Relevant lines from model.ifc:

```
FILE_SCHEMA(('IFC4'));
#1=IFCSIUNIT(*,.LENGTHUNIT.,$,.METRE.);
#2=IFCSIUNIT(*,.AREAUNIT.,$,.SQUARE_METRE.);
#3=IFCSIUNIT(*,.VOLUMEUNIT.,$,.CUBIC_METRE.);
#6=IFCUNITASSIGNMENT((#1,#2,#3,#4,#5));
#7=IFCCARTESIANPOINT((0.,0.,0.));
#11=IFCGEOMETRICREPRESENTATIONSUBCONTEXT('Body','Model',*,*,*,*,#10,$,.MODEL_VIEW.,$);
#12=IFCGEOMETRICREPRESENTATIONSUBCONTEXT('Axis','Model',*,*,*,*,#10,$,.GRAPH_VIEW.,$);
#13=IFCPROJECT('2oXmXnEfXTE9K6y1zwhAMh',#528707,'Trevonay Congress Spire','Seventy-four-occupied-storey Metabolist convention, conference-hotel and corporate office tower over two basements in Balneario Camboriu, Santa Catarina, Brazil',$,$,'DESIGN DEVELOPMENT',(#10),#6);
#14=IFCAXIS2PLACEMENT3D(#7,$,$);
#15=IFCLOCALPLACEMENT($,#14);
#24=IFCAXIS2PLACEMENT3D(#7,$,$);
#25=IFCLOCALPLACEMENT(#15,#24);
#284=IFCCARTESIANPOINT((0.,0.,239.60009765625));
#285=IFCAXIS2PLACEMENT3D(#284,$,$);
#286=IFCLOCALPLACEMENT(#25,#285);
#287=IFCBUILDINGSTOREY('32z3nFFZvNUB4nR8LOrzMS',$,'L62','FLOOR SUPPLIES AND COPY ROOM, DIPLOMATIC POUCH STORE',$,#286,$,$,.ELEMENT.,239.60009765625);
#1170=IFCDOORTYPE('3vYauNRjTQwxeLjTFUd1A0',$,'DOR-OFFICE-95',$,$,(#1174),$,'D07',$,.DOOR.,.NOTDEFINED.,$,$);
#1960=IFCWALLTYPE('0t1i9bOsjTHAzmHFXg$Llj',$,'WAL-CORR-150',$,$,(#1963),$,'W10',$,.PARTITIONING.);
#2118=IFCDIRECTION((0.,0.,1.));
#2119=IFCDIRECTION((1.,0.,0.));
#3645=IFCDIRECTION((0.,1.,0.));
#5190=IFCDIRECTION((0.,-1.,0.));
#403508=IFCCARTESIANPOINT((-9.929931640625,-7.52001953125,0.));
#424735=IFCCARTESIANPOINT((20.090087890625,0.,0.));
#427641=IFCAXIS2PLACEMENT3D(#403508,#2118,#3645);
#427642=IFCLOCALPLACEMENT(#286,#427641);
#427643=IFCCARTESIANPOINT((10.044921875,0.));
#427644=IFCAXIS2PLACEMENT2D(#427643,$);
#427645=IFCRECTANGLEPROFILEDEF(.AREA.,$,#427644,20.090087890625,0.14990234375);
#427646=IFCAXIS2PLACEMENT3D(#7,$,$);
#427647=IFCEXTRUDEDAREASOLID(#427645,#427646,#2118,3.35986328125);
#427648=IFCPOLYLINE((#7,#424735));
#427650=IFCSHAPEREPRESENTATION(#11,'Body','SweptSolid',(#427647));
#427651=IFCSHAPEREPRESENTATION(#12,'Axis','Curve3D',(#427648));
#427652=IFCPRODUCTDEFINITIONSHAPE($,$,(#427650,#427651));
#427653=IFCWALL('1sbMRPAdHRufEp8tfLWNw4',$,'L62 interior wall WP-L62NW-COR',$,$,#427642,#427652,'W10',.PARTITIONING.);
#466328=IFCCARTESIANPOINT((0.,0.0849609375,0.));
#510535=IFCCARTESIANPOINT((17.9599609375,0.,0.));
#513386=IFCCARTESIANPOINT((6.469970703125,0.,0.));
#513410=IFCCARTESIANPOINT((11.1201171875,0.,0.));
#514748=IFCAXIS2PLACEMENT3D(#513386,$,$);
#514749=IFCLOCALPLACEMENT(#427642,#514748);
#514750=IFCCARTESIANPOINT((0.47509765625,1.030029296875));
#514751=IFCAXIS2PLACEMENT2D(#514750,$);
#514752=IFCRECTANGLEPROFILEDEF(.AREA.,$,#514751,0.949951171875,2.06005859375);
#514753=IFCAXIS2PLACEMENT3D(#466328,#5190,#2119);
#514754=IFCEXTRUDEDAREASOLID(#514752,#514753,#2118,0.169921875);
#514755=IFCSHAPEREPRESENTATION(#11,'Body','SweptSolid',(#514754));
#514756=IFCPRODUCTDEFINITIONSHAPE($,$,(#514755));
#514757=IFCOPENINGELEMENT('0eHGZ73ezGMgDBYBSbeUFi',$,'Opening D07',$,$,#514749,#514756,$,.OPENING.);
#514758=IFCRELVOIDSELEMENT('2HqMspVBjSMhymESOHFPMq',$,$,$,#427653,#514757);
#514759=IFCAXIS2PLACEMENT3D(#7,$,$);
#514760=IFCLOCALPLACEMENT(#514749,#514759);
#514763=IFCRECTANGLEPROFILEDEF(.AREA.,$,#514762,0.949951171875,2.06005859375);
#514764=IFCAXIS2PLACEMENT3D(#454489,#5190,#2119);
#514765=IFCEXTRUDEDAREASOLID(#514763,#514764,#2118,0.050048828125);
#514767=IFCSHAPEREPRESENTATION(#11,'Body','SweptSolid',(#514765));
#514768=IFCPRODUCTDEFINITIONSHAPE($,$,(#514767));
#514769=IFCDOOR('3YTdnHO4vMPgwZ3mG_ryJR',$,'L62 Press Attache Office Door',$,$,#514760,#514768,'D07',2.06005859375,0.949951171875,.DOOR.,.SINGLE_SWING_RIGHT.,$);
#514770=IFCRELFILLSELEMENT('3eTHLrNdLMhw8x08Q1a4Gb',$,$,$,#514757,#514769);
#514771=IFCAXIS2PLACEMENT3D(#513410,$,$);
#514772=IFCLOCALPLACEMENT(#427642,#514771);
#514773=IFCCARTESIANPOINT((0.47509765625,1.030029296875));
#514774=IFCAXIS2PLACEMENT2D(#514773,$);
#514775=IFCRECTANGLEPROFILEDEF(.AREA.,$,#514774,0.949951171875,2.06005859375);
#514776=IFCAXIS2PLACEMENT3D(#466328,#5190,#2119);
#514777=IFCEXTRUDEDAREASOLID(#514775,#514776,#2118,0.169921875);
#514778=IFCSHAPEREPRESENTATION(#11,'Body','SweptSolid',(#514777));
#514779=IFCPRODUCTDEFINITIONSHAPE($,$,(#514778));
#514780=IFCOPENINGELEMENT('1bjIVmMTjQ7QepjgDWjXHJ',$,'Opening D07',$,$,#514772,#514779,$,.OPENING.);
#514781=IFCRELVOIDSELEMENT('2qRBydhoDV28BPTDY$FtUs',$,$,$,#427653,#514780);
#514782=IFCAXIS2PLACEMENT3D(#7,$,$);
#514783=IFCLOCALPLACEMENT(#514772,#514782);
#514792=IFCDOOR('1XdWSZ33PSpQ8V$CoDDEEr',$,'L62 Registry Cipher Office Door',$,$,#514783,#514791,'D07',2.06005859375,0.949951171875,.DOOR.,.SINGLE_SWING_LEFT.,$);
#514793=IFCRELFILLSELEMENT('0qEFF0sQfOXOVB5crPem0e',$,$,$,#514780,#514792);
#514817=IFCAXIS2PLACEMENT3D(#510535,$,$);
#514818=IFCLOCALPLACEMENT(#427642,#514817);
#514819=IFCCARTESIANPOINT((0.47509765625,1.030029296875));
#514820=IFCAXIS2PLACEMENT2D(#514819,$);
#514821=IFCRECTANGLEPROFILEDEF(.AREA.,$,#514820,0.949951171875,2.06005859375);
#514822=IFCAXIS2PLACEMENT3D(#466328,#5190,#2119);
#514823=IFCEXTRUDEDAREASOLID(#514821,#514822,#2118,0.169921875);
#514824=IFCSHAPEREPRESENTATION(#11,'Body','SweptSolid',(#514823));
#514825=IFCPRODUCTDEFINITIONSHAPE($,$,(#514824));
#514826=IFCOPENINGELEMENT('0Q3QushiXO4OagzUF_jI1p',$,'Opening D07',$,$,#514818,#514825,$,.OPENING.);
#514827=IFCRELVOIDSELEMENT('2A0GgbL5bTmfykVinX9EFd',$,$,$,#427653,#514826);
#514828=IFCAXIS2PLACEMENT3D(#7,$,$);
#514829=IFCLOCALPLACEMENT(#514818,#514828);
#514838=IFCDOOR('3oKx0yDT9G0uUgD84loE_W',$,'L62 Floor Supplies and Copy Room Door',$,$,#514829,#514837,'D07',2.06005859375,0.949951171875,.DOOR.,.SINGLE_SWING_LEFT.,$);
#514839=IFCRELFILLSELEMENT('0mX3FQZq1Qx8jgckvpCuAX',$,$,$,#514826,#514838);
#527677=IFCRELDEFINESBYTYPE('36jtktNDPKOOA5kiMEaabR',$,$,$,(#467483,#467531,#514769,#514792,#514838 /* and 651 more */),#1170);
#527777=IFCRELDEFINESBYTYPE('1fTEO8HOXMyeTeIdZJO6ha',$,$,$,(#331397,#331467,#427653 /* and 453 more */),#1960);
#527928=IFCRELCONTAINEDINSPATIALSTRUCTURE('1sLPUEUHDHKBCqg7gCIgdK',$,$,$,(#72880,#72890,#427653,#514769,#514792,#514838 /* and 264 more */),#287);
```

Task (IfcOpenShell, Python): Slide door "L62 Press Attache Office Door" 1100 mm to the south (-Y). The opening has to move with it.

```python
import ifcopenshell
import ifcopenshell.api.geometry
import ifcopenshell.util.placement
import ifcopenshell.util.unit

model = ifcopenshell.open("model.ifc")
unit_scale = ifcopenshell.util.unit.calculate_unit_scale(model)

door = model.by_id(514769)
opening = door.FillsVoids[0].RelatingOpeningElement
wall = opening.VoidsElements[0].RelatingBuildingElement

wall_matrix = ifcopenshell.util.placement.get_local_placement(wall.ObjectPlacement)
shift = wall_matrix[:3, 0] * -1.1 / unit_scale
before = ifcopenshell.util.placement.get_local_placement(door.ObjectPlacement)[:3, 3].copy()

# The door is placed relative to its opening, so it follows when the opening moves.
matrix = ifcopenshell.util.placement.get_local_placement(opening.ObjectPlacement)
matrix[:3, 3] += shift
ifcopenshell.api.geometry.edit_object_placement(
    model, product=opening, matrix=matrix, is_si=False, should_transform_children=True
)

after = ifcopenshell.util.placement.get_local_placement(door.ObjectPlacement)[:3, 3]
print("door moved by", (after - before).round(3) + 0.0)

model.write("model_edited.ifc")
```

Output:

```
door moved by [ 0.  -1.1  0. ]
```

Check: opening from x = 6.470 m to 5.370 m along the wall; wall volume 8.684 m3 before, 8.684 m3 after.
